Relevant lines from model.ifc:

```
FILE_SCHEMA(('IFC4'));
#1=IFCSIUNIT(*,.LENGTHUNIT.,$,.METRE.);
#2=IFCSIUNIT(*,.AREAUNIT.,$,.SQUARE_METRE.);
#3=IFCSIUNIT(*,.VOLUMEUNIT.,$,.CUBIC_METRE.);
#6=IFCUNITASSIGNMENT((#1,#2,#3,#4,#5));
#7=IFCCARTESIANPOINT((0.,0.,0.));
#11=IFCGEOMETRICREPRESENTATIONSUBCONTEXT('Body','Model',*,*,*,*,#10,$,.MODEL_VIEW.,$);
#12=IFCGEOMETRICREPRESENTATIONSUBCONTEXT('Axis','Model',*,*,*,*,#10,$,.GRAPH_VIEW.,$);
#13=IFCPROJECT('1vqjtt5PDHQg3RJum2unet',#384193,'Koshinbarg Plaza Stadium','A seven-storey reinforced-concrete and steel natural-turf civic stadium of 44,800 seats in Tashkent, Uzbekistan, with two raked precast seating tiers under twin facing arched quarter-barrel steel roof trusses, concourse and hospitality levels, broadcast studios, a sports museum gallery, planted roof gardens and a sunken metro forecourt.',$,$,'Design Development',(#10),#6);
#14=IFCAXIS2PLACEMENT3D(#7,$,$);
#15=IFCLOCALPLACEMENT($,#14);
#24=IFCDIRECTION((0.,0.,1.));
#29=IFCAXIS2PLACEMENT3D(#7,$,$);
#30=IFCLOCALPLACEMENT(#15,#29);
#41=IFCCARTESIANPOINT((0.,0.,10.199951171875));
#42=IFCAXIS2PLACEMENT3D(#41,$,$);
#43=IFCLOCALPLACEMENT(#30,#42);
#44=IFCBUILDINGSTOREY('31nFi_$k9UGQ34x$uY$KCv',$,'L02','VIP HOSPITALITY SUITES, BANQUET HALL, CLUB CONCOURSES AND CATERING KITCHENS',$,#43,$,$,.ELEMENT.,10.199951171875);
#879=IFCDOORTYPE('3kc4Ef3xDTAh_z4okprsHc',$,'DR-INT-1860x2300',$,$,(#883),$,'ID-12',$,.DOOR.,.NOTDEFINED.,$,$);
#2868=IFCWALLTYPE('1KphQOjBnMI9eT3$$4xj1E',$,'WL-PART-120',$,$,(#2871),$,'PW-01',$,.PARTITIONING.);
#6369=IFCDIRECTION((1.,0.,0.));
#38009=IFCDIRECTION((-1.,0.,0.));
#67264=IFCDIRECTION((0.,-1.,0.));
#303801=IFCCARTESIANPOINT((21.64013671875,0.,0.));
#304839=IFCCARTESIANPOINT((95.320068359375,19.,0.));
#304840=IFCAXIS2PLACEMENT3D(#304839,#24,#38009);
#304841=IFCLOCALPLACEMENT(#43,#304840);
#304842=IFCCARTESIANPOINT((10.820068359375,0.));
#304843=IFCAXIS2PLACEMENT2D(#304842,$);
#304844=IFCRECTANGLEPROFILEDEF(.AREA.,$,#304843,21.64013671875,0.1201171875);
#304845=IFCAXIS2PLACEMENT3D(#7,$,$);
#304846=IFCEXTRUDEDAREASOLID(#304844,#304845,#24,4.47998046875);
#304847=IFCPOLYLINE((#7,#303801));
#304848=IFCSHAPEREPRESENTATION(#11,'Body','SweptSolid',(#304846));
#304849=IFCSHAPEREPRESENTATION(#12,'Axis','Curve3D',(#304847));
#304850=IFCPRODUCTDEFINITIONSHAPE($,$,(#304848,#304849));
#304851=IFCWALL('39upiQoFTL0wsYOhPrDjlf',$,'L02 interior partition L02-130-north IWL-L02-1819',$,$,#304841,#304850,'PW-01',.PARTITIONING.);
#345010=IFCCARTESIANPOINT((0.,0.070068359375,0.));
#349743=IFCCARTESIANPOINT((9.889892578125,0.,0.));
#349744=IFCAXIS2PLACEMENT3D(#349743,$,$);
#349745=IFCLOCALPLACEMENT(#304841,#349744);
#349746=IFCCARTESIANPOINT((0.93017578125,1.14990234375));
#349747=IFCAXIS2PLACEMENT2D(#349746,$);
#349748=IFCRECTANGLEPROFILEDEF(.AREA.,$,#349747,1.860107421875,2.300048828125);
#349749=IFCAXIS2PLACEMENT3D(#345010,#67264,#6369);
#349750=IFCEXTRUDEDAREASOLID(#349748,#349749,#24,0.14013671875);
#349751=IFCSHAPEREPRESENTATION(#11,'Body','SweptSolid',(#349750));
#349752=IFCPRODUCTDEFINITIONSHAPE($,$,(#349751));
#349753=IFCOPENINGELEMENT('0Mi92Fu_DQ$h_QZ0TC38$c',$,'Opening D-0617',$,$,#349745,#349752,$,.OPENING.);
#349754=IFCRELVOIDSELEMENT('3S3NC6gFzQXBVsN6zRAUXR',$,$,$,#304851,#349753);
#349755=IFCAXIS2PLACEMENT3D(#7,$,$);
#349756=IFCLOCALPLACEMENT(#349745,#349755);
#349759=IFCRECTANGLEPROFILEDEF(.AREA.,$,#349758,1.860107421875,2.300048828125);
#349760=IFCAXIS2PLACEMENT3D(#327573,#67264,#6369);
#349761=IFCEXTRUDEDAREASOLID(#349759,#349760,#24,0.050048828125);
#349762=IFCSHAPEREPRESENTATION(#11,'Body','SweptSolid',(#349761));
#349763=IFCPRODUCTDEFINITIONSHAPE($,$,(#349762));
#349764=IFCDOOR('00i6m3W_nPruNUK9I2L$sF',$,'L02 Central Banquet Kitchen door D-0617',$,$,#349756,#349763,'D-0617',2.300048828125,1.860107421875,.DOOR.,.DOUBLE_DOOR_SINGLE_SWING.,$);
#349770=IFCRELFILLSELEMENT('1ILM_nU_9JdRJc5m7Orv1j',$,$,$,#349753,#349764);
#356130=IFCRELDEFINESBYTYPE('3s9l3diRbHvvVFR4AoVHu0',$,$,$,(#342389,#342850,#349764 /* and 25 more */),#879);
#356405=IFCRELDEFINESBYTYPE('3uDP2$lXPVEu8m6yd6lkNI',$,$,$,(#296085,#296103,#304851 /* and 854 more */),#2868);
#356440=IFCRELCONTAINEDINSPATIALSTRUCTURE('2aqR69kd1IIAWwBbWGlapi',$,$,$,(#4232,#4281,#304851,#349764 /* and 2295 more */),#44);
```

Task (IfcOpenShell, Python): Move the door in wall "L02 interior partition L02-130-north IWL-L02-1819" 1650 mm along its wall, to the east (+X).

```python
import ifcopenshell
import ifcopenshell.api.geometry
import ifcopenshell.util.placement
import ifcopenshell.util.unit

model = ifcopenshell.open("model.ifc")
unit_scale = ifcopenshell.util.unit.calculate_unit_scale(model)

door = model.by_guid("00i6m3W_nPruNUK9I2L$sF")
opening = door.FillsVoids[0].RelatingOpeningElement
wall = opening.VoidsElements[0].RelatingBuildingElement

wall_matrix = ifcopenshell.util.placement.get_local_placement(wall.ObjectPlacement)
shift = wall_matrix[:3, 0] * -1.65 / unit_scale
before = ifcopenshell.util.placement.get_local_placement(door.ObjectPlacement)[:3, 3].copy()

# The door is placed relative to its opening, so it follows when the opening moves.
matrix = ifcopenshell.util.placement.get_local_placement(opening.ObjectPlacement)
matrix[:3, 3] += shift
ifcopenshell.api.geometry.edit_object_placement(
    model, product=opening, matrix=matrix, is_si=False, should_transform_children=True
)

after = ifcopenshell.util.placement.get_local_placement(door.ObjectPlacement)[:3, 3]
print("door moved by", (after - before).round(3) + 0.0)

model.write("model_rev.ifc")
```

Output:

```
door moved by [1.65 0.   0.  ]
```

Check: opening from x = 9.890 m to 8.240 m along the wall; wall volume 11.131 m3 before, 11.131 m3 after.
